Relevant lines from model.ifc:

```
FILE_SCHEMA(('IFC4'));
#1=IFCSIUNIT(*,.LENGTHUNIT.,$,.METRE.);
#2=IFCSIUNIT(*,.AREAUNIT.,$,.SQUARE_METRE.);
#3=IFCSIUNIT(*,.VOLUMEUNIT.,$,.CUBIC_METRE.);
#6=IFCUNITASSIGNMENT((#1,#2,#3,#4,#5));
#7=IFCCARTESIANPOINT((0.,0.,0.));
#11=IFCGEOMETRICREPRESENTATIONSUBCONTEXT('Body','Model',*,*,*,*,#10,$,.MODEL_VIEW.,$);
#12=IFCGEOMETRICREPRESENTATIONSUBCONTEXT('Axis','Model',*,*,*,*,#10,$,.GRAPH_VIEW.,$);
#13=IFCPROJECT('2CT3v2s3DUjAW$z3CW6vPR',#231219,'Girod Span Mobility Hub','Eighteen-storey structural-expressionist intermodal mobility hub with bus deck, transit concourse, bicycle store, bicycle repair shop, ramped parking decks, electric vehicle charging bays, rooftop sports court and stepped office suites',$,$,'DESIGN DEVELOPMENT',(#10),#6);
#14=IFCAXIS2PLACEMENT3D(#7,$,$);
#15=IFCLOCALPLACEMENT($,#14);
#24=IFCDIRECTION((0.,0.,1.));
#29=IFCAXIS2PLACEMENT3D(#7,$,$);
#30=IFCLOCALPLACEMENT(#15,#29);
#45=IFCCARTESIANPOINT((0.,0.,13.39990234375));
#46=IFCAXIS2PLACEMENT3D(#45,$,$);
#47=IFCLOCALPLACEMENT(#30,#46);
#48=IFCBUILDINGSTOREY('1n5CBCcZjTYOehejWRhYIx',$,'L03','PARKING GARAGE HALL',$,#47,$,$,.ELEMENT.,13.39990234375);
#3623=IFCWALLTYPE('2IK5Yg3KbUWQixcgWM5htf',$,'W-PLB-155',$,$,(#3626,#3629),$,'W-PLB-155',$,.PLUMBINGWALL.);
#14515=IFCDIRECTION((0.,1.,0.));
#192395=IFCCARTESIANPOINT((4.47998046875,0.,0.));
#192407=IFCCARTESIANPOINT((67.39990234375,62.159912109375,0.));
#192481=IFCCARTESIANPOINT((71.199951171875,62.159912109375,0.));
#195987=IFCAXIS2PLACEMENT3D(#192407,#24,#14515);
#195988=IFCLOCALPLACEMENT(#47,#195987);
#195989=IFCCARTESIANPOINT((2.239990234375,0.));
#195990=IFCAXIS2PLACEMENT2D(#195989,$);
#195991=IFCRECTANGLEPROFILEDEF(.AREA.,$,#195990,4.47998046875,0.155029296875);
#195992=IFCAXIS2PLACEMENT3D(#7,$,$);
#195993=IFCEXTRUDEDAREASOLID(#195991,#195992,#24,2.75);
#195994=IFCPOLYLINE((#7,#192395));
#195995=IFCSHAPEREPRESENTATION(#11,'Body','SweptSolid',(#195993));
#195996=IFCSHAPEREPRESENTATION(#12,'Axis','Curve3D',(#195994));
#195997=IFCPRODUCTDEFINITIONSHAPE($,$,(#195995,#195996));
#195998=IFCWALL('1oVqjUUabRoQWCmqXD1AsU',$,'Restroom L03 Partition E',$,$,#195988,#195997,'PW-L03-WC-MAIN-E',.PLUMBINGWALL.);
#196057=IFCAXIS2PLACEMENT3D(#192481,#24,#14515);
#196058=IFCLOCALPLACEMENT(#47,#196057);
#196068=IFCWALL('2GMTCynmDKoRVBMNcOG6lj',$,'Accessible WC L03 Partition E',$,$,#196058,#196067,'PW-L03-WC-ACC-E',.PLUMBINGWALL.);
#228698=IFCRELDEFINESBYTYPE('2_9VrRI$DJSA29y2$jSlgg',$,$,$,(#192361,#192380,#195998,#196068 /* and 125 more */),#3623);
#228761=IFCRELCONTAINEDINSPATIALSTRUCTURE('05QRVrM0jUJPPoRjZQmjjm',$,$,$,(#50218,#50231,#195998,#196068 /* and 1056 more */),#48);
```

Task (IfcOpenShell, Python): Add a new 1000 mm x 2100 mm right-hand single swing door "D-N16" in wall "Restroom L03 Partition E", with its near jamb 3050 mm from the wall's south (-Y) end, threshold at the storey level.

```python
import numpy as np
import ifcopenshell
import ifcopenshell.api.feature
import ifcopenshell.api.geometry
import ifcopenshell.api.root
import ifcopenshell.api.spatial
import ifcopenshell.geom
import ifcopenshell.util.element
import ifcopenshell.util.placement
import ifcopenshell.util.representation
import ifcopenshell.util.shape
import ifcopenshell.util.unit

model = ifcopenshell.open("model.ifc")
unit_scale = ifcopenshell.util.unit.calculate_unit_scale(model)
settings = ifcopenshell.geom.settings()


def volume(element):
    """Net volume in cubic metres, openings subtracted."""
    shape = ifcopenshell.geom.create_shape(settings, element)
    return ifcopenshell.util.shape.get_volume(shape.geometry)


wall = model.by_guid("1oVqjUUabRoQWCmqXD1AsU")
storey = ifcopenshell.util.element.get_container(wall, ifc_class="IfcBuildingStorey")
context = ifcopenshell.util.representation.get_context(model, "Model", "Body", "MODEL_VIEW")
before = volume(wall)

width, height, from_end, sill = 1, 2.1, 3.05, 0.0  # metres

# The wall runs along its own X axis, and the end named is its -X end.
wall_shape = ifcopenshell.geom.create_shape(settings, wall)
x, y, z = ifcopenshell.util.shape.get_vertices(wall_shape.geometry).T
start = x.min() + from_end
face, thickness = float(y.min()), float(y.max() - y.min())
wall_matrix = ifcopenshell.util.placement.get_local_placement(wall.ObjectPlacement)
level = ifcopenshell.util.placement.get_local_placement(storey.ObjectPlacement)[2, 3]


def in_wall(x, y):
    """Placement at x, y metres in the wall's axes, at sill height."""
    matrix = wall_matrix.copy()
    matrix[:, 3] = wall_matrix @ np.array([x / unit_scale, y / unit_scale, 0.0, 1.0])
    matrix[2, 3] = level + sill / unit_scale
    return matrix


# Opening: a box that overshoots both wall faces by 50 mm.
opening = ifcopenshell.api.root.create_entity(model, ifc_class="IfcOpeningElement", predefined_type="OPENING")
box = ifcopenshell.api.geometry.add_wall_representation(
    model, context=context, length=width, height=height, thickness=thickness + 0.1
)
ifcopenshell.api.geometry.assign_representation(model, product=opening, representation=box)
ifcopenshell.api.geometry.edit_object_placement(model, product=opening, matrix=in_wall(start, face - 0.05), is_si=False)
ifcopenshell.api.feature.add_feature(model, feature=opening, element=wall)

door = ifcopenshell.api.root.create_entity(model, ifc_class="IfcDoor", name="D-N16", predefined_type="DOOR")
door.OverallWidth, door.OverallHeight = width / unit_scale, height / unit_scale
door.OperationType = "SINGLE_SWING_RIGHT"
body = ifcopenshell.api.geometry.add_door_representation(
    model,
    context=context,
    overall_width=door.OverallWidth,
    overall_height=door.OverallHeight,
    operation_type="SINGLE_SWING_RIGHT",
    lining_properties={"LiningDepth": thickness / unit_scale, "ThresholdDepth": thickness / unit_scale},
)
ifcopenshell.api.geometry.assign_representation(model, product=door, representation=body)
ifcopenshell.api.spatial.assign_container(model, products=[door], relating_structure=storey)
ifcopenshell.api.feature.add_filling(model, opening=opening, element=door)

# The lining spans the wall, so the door starts at the wall face.
ifcopenshell.api.geometry.edit_object_placement(model, product=door, matrix=in_wall(start, face), is_si=False)

after = volume(wall)

print(f"wall volume {before:.3f} -> {after:.3f} m3")

model.write("model_rev.ifc")
```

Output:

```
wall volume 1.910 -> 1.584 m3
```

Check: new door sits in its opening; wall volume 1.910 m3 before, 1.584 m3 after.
